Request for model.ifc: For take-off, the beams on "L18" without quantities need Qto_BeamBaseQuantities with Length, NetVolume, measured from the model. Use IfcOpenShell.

First a look at what the model holds.

```python
import ifcopenshell
import ifcopenshell.util.element
import ifcopenshell.util.unit

model = ifcopenshell.open("model.ifc")
print(model.schema)
for unit_type in ("LENGTHUNIT", "AREAUNIT", "VOLUMEUNIT"):
    print(unit_type, ifcopenshell.util.unit.calculate_unit_scale(model, unit_type))
storey = next(s for s in model.by_type("IfcBuildingStorey") if s.Name == "L18")
beams = [e for e in ifcopenshell.util.element.get_decomposition(storey) if e.is_a("IfcBeam")]
for e in sorted(beams, key=lambda e: e.id()):
    print(e.id(), e.is_a(), e.Name, list(ifcopenshell.util.element.get_psets(e, qtos_only=True)), sep=" | ")
```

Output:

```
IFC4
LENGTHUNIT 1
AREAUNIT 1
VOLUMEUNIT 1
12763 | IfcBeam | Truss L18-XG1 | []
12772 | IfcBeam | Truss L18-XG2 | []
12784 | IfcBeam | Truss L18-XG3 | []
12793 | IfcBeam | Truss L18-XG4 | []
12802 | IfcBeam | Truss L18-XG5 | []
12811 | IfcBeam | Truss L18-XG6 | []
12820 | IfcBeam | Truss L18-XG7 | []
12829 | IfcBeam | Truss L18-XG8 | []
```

```python
import ifcopenshell
import ifcopenshell.api.pset
import ifcopenshell.geom
import ifcopenshell.util.element
import ifcopenshell.util.shape
import ifcopenshell.util.unit

model = ifcopenshell.open("model.ifc")
unit_scale = ifcopenshell.util.unit.calculate_unit_scale(model)
volume_scale = ifcopenshell.util.unit.calculate_unit_scale(model, "VOLUMEUNIT")
settings = ifcopenshell.geom.settings()

storey = next(s for s in model.by_type("IfcBuildingStorey") if s.Name == "L18")
beams = [e for e in ifcopenshell.util.element.get_decomposition(storey) if e.is_a("IfcBeam")]

for e in sorted(beams, key=lambda e: e.id()):
    if ifcopenshell.util.element.get_psets(e, qtos_only=True, should_inherit=False):
        continue
    # Geometry comes back in metres, in the element's own axes.
    shape = ifcopenshell.geom.create_shape(settings, e)
    values = {
        "Length": ifcopenshell.util.shape.get_max_xyz(shape.geometry) / unit_scale,
        "NetVolume": ifcopenshell.util.shape.get_volume(shape.geometry) / volume_scale,
    }
    qto = ifcopenshell.api.pset.add_qto(model, product=e, name="Qto_BeamBaseQuantities")
    ifcopenshell.api.pset.edit_qto(model, qto=qto, properties=values)
    print(e.id(), {k: round(v, 3) for k, v in values.items()})

model.write("model_rev.ifc")
```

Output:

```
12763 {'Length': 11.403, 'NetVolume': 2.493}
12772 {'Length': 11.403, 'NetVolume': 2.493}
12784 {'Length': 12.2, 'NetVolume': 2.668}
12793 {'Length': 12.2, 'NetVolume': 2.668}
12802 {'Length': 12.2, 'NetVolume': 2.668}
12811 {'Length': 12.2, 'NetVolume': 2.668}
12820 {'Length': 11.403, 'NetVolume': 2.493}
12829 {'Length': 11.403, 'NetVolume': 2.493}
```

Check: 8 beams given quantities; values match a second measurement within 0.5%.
